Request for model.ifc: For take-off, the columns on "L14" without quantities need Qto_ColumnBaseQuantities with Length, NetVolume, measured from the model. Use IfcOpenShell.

First a look at what the model holds.

```python
import ifcopenshell
import ifcopenshell.util.element
import ifcopenshell.util.unit

model = ifcopenshell.open("model.ifc")
print(model.schema)
for unit_type in ("LENGTHUNIT", "AREAUNIT", "VOLUMEUNIT"):
    print(unit_type, ifcopenshell.util.unit.calculate_unit_scale(model, unit_type))
storey = next(s for s in model.by_type("IfcBuildingStorey") if s.Name == "L14")
columns = [e for e in ifcopenshell.util.element.get_decomposition(storey) if e.is_a("IfcColumn")]
for e in sorted(columns, key=lambda e: e.id()):
    print(e.id(), e.is_a(), e.Name, list(ifcopenshell.util.element.get_psets(e, qtos_only=True)), sep=" | ")
```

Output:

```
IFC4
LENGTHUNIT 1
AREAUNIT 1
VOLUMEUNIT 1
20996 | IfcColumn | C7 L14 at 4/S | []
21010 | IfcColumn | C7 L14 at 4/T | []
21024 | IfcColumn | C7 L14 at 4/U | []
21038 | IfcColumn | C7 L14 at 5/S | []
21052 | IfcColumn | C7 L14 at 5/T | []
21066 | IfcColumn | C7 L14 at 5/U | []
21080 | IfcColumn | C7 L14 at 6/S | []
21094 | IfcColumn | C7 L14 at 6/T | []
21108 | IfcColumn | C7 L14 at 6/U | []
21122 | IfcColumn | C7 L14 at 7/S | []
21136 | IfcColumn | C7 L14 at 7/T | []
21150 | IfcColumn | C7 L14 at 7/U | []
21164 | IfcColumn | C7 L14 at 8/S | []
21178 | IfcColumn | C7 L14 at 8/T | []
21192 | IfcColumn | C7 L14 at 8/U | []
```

```python
import ifcopenshell
import ifcopenshell.api.pset
import ifcopenshell.geom
import ifcopenshell.util.element
import ifcopenshell.util.shape
import ifcopenshell.util.unit

model = ifcopenshell.open("model.ifc")
unit_scale = ifcopenshell.util.unit.calculate_unit_scale(model)
volume_scale = ifcopenshell.util.unit.calculate_unit_scale(model, "VOLUMEUNIT")
settings = ifcopenshell.geom.settings()

storey = next(s for s in model.by_type("IfcBuildingStorey") if s.Name == "L14")
columns = [e for e in ifcopenshell.util.element.get_decomposition(storey) if e.is_a("IfcColumn")]

for e in sorted(columns, key=lambda e: e.id()):
    if ifcopenshell.util.element.get_psets(e, qtos_only=True, should_inherit=False):
        continue
    # Geometry comes back in metres, in the element's own axes.
    shape = ifcopenshell.geom.create_shape(settings, e)
    values = {
        "Length": ifcopenshell.util.shape.get_z(shape.geometry) / unit_scale,
        "NetVolume": ifcopenshell.util.shape.get_volume(shape.geometry) / volume_scale,
    }
    qto = ifcopenshell.api.pset.add_qto(model, product=e, name="Qto_ColumnBaseQuantities")
    ifcopenshell.api.pset.edit_qto(model, qto=qto, properties=values)
    print(e.id(), {k: round(v, 3) for k, v in values.items()})

model.write("model-out.ifc")
```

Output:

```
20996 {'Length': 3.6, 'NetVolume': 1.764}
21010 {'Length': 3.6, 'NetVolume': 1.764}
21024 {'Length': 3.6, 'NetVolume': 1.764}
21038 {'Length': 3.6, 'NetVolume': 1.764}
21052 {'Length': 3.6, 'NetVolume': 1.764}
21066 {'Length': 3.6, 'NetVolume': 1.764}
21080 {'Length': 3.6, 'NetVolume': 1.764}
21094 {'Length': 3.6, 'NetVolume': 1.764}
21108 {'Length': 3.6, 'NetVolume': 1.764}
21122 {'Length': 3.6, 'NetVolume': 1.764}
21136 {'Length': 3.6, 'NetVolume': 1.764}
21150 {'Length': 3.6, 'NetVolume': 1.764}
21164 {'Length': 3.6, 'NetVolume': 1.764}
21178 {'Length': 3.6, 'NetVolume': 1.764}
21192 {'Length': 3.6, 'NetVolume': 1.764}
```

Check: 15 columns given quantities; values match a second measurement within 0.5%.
